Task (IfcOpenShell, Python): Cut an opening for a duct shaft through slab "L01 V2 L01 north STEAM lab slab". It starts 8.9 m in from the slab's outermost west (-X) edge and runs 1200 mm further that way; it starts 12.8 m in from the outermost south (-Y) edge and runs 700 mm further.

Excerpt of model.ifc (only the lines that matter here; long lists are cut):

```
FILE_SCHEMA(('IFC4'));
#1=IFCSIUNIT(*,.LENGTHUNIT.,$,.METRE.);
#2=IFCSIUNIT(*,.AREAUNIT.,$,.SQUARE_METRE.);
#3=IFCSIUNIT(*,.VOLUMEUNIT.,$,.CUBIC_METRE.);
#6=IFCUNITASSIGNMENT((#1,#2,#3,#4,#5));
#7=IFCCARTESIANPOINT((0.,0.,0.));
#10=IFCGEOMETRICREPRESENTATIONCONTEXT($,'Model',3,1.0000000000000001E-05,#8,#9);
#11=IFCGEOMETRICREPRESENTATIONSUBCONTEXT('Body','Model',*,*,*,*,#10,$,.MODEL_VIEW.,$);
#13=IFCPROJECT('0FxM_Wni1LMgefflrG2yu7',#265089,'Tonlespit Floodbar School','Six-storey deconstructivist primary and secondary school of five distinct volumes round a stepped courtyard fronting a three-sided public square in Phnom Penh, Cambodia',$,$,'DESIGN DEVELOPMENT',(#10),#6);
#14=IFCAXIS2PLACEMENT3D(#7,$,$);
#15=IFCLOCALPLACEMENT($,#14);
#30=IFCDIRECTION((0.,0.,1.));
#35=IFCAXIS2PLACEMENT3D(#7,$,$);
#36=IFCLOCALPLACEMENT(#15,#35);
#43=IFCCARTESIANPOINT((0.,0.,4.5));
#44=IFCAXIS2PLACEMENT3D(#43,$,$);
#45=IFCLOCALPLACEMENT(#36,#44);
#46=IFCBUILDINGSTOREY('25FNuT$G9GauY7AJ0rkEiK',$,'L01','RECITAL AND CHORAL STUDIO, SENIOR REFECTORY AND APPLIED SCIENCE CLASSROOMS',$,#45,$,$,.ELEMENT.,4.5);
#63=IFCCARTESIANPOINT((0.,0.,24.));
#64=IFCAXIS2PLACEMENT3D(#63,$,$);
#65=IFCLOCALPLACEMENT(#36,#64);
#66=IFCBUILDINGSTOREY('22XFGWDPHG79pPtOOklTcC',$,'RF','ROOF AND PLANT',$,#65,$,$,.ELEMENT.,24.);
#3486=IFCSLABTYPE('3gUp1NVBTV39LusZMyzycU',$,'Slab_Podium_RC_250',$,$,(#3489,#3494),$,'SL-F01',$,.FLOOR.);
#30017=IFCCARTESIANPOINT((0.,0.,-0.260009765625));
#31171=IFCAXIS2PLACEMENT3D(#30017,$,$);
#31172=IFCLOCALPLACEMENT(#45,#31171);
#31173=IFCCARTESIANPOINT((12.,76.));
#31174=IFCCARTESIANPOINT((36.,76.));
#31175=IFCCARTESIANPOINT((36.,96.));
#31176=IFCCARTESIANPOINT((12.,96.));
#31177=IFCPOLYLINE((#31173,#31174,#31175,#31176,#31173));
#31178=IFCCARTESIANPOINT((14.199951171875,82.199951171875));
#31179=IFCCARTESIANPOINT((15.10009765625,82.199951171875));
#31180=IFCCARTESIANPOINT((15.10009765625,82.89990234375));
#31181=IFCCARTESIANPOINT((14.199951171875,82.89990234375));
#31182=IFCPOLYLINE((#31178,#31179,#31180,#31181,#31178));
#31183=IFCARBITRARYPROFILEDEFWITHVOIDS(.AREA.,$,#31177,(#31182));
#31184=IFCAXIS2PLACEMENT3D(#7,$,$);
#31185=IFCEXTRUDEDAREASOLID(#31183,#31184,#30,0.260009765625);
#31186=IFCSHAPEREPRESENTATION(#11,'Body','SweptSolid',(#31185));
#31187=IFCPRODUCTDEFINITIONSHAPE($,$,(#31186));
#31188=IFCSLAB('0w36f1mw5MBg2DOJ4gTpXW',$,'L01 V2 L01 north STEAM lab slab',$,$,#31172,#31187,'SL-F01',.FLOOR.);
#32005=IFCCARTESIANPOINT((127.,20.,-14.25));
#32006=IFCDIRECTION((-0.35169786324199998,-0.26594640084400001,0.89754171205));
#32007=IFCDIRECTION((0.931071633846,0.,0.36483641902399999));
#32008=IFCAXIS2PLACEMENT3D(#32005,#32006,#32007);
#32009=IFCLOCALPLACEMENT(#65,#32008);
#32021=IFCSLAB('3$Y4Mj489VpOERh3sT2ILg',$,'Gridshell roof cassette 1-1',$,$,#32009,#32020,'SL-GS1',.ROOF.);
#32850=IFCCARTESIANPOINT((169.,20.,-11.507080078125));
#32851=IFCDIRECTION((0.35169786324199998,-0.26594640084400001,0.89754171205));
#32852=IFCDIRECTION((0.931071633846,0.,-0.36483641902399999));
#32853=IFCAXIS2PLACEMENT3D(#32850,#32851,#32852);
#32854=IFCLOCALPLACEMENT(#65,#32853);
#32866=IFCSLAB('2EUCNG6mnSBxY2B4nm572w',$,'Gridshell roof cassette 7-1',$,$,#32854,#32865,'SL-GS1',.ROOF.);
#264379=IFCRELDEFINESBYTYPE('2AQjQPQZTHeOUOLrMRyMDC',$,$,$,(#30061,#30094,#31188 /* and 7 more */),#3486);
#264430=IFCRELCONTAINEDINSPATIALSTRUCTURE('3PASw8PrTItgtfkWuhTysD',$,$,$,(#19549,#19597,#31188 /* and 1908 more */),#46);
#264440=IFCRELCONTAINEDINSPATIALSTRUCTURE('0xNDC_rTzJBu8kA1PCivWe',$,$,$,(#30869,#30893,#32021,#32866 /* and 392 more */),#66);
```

```python
import numpy as np
import ifcopenshell
import ifcopenshell.api.feature
import ifcopenshell.api.geometry
import ifcopenshell.api.root
import ifcopenshell.geom
import ifcopenshell.util.placement
import ifcopenshell.util.representation
import ifcopenshell.util.shape
import ifcopenshell.util.unit

model = ifcopenshell.open("model.ifc")
unit_scale = ifcopenshell.util.unit.calculate_unit_scale(model)
settings = ifcopenshell.geom.settings()


def volume(element):
    """Net volume in cubic metres, openings subtracted."""
    shape = ifcopenshell.geom.create_shape(settings, element)
    return ifcopenshell.util.shape.get_volume(shape.geometry)


slab = model.by_id(31188)
before = volume(slab)

# Extent in the slab's own axes, in metres. The edges named are its -X and -Y sides.
slab_shape = ifcopenshell.geom.create_shape(settings, slab)
vertices = ifcopenshell.util.shape.get_vertices(slab_shape.geometry)
x_min, y_min, bottom = vertices.min(axis=0)
top = vertices[:, 2].max()

opening = ifcopenshell.api.root.create_entity(model, ifc_class="IfcOpeningElement", name="Duct shaft opening", predefined_type="OPENING")
context = ifcopenshell.util.representation.get_context(model, "Model", "Body", "MODEL_VIEW")
width, depth = 1.2, 0.7
outline = [(0.0, 0.0), (width, 0.0), (width, depth), (0.0, depth), (0.0, 0.0)]
# Overshoot both faces by 50 mm so the cut is clean.
shape = ifcopenshell.api.geometry.add_slab_representation(
    model, context=context, depth=top - bottom + 0.1, polyline=outline
)
ifcopenshell.api.geometry.assign_representation(model, product=opening, representation=shape)

matrix = ifcopenshell.util.placement.get_local_placement(slab.ObjectPlacement)
matrix[:, 3] = matrix @ np.append(np.array([x_min + 8.9, y_min + 12.8, bottom - 0.05]) / unit_scale, 1.0)
ifcopenshell.api.geometry.edit_object_placement(model, product=opening, matrix=matrix, is_si=False)
ifcopenshell.api.feature.add_feature(model, feature=opening, element=slab)

after = volume(slab)

print(f"slab volume {before:.3f} -> {after:.3f} m3")

model.write("model_rev.ifc")
```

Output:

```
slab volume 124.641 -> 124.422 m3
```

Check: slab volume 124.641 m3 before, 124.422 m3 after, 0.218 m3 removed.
